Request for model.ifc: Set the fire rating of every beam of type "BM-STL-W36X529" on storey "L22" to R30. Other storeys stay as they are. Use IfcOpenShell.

First a look at what the model holds.

```python
import ifcopenshell
import ifcopenshell.util.element

model = ifcopenshell.open("model.ifc")
print(model.schema)
storey = next(s for s in model.by_type("IfcBuildingStorey") if s.Name == "L22")
beams = [e for e in ifcopenshell.util.element.get_decomposition(storey) if e.is_a("IfcBeam")]
seen = {}
for e in beams:
    element_type = ifcopenshell.util.element.get_type(e)
    key = (element_type.Name if element_type != e and element_type else None, ifcopenshell.util.element.get_pset(e, "Pset_BeamCommon", "FireRating"))
    seen[key] = seen.get(key, 0) + 1
for (name, value), count in sorted(seen.items(), key=str):
    print(count, "x", name, "|", value)
```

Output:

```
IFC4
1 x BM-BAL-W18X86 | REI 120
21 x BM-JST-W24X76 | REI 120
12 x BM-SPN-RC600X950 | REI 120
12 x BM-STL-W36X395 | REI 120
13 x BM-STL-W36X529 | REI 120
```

```python
import ifcopenshell
import ifcopenshell.api.pset
import ifcopenshell.util.element

model = ifcopenshell.open("model.ifc")

storey = next(s for s in model.by_type("IfcBuildingStorey") if s.Name == "L22")
beams = [e for e in ifcopenshell.util.element.get_decomposition(storey) if e.is_a("IfcBeam")]

count = 0
for e in beams:
    element_type = ifcopenshell.util.element.get_type(e)
    if element_type in (None, e) or element_type.Name != "BM-STL-W36X529":
        continue
    # add_pset returns the element's existing set when there is one.
    pset = ifcopenshell.api.pset.add_pset(model, product=e, name="Pset_BeamCommon")
    ifcopenshell.api.pset.edit_pset(model, pset=pset, properties={"FireRating": "R30"})
    count += 1

print(count, "beams updated")

model.write("model-out.ifc")
```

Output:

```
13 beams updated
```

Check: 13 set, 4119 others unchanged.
